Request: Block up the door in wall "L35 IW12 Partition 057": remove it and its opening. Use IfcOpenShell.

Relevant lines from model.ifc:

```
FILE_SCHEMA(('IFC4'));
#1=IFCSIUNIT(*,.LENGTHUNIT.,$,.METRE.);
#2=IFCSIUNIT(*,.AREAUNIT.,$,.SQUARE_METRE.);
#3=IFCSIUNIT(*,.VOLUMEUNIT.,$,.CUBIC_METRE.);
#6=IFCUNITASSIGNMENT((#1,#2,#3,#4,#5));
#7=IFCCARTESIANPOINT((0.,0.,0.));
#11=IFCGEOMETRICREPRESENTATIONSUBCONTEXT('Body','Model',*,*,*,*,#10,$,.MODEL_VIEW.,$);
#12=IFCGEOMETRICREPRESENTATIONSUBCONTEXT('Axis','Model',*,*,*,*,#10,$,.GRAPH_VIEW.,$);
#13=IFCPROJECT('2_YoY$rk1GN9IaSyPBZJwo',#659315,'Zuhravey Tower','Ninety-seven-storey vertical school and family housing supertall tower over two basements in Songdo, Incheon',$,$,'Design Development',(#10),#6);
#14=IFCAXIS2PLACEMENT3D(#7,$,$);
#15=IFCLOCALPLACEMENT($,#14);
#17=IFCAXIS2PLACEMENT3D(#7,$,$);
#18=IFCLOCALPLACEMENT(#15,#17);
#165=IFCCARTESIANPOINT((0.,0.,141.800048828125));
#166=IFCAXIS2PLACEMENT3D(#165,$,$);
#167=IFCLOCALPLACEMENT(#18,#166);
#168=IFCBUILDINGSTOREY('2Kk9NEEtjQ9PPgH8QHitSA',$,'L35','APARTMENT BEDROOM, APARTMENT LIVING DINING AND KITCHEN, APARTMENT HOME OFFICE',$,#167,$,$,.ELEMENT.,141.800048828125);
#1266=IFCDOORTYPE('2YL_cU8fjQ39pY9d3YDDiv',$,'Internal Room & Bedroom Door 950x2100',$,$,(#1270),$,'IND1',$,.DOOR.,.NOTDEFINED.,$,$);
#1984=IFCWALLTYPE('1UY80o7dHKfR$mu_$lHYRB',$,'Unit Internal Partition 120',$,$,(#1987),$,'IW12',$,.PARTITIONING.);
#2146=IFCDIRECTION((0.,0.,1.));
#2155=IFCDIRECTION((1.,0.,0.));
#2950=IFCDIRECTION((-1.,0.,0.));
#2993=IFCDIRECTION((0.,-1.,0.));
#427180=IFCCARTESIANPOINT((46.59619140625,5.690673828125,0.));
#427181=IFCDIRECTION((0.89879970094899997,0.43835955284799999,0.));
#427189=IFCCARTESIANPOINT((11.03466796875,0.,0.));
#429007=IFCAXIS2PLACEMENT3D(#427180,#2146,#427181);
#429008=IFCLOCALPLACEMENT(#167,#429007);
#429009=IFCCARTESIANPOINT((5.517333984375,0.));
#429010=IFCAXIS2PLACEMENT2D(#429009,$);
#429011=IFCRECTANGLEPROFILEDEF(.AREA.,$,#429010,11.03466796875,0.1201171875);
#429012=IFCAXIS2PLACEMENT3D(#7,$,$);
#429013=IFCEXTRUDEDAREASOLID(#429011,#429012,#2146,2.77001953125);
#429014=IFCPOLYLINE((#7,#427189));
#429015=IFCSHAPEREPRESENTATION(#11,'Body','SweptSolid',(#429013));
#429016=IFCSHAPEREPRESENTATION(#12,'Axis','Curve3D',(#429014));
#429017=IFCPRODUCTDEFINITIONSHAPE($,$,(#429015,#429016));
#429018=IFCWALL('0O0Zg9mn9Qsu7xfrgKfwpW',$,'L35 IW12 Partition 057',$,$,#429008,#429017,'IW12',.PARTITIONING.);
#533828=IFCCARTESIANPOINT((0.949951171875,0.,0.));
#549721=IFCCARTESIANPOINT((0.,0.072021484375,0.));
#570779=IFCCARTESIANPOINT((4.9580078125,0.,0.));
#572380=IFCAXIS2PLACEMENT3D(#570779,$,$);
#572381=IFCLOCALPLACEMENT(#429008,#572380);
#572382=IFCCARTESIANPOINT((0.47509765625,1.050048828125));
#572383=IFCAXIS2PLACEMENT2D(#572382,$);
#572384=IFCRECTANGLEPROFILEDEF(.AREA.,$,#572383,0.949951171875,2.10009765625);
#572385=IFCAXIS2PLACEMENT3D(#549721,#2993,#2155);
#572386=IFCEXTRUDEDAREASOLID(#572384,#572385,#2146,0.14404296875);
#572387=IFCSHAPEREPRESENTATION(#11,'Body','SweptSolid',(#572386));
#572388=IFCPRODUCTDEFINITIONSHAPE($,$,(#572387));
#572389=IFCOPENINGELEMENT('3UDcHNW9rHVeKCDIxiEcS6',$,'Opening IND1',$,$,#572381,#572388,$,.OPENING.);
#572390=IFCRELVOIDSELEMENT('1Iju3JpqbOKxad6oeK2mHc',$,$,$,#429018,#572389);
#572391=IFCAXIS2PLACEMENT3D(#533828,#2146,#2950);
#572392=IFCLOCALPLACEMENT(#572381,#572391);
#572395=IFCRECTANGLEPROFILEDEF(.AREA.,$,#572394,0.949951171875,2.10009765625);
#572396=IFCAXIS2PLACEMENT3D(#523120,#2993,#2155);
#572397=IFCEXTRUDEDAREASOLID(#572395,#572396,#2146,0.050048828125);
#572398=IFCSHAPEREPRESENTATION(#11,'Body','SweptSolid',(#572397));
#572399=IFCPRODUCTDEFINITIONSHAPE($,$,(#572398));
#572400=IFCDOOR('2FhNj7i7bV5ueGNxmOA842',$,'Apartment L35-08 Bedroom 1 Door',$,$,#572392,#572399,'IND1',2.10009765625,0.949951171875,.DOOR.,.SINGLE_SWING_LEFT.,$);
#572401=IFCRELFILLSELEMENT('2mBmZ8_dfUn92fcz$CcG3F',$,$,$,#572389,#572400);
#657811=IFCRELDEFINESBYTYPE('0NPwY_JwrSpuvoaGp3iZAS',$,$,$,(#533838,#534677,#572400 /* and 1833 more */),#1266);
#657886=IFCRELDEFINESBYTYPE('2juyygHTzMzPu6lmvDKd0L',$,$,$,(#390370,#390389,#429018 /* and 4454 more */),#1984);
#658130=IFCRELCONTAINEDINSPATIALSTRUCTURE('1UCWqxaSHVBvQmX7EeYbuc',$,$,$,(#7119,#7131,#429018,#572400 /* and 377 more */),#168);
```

```python
import ifcopenshell
import ifcopenshell.api.feature
import ifcopenshell.api.root
import ifcopenshell.geom
import ifcopenshell.util.shape

model = ifcopenshell.open("model.ifc")
settings = ifcopenshell.geom.settings()


def volume(element):
    """Net volume in cubic metres, openings subtracted."""
    shape = ifcopenshell.geom.create_shape(settings, element)
    return ifcopenshell.util.shape.get_volume(shape.geometry)


door = model.by_guid("2FhNj7i7bV5ueGNxmOA842")
opening = door.FillsVoids[0].RelatingOpeningElement
wall = opening.VoidsElements[0].RelatingBuildingElement
before = volume(wall)

ifcopenshell.api.root.remove_product(model, product=door)
ifcopenshell.api.feature.remove_feature(model, feature=opening)

after = volume(wall)

print(f"wall volume {before:.3f} -> {after:.3f} m3")

model.write("model-out.ifc")
```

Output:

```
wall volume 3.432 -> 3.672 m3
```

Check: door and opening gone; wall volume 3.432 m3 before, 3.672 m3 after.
